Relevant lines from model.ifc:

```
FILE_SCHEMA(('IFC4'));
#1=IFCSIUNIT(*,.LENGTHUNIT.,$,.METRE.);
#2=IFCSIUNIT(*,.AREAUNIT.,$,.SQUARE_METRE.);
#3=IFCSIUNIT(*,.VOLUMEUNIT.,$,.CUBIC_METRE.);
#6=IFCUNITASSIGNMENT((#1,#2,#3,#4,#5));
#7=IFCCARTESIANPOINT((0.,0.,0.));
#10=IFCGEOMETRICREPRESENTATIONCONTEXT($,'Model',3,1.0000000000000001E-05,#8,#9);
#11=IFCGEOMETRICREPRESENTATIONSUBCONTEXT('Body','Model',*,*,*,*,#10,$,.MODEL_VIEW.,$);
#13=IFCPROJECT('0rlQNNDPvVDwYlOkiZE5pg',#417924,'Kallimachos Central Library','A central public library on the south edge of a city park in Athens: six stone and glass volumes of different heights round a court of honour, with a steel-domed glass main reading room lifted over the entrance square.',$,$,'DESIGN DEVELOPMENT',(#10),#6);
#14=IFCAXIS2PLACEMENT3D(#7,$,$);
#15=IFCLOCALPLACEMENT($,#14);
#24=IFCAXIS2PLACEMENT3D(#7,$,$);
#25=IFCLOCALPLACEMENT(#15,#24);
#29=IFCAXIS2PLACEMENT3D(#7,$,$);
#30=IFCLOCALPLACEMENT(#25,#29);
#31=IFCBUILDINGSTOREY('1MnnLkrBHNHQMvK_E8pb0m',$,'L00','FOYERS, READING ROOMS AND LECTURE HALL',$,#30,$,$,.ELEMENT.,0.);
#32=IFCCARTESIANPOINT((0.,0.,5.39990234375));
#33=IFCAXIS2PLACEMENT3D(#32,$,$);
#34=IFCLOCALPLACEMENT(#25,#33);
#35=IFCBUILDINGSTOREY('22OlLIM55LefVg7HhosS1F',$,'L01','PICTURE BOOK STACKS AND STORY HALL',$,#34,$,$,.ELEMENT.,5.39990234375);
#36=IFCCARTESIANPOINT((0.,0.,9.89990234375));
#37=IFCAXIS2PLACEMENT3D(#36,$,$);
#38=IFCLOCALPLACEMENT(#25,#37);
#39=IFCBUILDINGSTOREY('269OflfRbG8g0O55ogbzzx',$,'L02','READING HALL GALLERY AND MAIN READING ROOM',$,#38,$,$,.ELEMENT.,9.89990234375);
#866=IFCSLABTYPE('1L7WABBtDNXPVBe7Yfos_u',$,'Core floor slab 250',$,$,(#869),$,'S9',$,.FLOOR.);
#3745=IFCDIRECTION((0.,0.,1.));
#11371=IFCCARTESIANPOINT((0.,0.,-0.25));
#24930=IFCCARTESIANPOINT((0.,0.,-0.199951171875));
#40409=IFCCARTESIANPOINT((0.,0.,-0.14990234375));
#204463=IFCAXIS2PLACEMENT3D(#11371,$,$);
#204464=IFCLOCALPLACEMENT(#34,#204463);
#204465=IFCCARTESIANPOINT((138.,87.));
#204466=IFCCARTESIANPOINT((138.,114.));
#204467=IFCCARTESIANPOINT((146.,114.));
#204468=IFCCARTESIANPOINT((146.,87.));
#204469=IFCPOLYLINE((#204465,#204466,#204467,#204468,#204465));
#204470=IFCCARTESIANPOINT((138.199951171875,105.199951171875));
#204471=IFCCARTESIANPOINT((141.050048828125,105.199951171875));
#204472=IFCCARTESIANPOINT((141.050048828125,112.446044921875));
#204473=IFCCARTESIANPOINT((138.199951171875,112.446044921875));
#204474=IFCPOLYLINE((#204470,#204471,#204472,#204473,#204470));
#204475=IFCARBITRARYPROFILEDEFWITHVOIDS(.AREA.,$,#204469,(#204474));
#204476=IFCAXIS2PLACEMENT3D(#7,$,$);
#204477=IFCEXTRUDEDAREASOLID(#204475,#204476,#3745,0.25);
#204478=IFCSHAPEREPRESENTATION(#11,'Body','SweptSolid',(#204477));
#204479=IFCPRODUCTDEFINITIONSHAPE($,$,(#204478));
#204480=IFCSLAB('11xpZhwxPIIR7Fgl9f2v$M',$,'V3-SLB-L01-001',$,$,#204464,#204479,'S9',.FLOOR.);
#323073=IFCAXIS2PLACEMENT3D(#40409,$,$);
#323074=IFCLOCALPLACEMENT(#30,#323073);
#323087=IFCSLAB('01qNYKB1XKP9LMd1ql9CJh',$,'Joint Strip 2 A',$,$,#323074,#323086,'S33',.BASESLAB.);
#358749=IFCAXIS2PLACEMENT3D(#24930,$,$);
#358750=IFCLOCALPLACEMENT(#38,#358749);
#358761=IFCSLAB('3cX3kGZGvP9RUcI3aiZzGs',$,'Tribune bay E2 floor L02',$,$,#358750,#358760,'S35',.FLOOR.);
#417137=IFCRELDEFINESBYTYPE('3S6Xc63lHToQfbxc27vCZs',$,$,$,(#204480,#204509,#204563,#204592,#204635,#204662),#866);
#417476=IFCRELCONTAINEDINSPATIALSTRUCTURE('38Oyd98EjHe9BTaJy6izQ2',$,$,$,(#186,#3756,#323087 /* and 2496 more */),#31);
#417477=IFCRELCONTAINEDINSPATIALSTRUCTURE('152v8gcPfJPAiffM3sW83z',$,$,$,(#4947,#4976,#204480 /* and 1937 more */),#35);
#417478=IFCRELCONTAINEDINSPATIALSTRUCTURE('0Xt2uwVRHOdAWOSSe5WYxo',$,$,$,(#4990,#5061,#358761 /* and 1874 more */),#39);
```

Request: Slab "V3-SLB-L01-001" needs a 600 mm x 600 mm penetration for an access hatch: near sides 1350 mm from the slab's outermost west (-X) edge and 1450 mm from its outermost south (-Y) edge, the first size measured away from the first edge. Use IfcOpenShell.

```python
import numpy as np
import ifcopenshell
import ifcopenshell.api.feature
import ifcopenshell.api.geometry
import ifcopenshell.api.root
import ifcopenshell.geom
import ifcopenshell.util.placement
import ifcopenshell.util.representation
import ifcopenshell.util.shape
import ifcopenshell.util.unit

model = ifcopenshell.open("model.ifc")
unit_scale = ifcopenshell.util.unit.calculate_unit_scale(model)
settings = ifcopenshell.geom.settings()


def volume(element):
    """Net volume in cubic metres, openings subtracted."""
    shape = ifcopenshell.geom.create_shape(settings, element)
    return ifcopenshell.util.shape.get_volume(shape.geometry)


slab = model.by_id(204480)
before = volume(slab)

# Extent in the slab's own axes, in metres. The edges named are its -X and -Y sides.
slab_shape = ifcopenshell.geom.create_shape(settings, slab)
vertices = ifcopenshell.util.shape.get_vertices(slab_shape.geometry)
x_min, y_min, bottom = vertices.min(axis=0)
top = vertices[:, 2].max()

opening = ifcopenshell.api.root.create_entity(model, ifc_class="IfcOpeningElement", name="Access hatch opening", predefined_type="OPENING")
context = ifcopenshell.util.representation.get_context(model, "Model", "Body", "MODEL_VIEW")
width, depth = 0.6, 0.6
outline = [(0.0, 0.0), (width, 0.0), (width, depth), (0.0, depth), (0.0, 0.0)]
# Overshoot both faces by 50 mm so the cut is clean.
shape = ifcopenshell.api.geometry.add_slab_representation(
    model, context=context, depth=top - bottom + 0.1, polyline=outline
)
ifcopenshell.api.geometry.assign_representation(model, product=opening, representation=shape)

matrix = ifcopenshell.util.placement.get_local_placement(slab.ObjectPlacement)
matrix[:, 3] = matrix @ np.append(np.array([x_min + 1.35, y_min + 1.45, bottom - 0.05]) / unit_scale, 1.0)
ifcopenshell.api.geometry.edit_object_placement(model, product=opening, matrix=matrix, is_si=False)
ifcopenshell.api.feature.add_feature(model, feature=opening, element=slab)

after = volume(slab)

print(f"slab volume {before:.3f} -> {after:.3f} m3")

model.write("model_v2.ifc")
```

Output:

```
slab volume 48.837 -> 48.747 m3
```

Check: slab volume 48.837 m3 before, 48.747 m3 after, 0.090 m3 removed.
